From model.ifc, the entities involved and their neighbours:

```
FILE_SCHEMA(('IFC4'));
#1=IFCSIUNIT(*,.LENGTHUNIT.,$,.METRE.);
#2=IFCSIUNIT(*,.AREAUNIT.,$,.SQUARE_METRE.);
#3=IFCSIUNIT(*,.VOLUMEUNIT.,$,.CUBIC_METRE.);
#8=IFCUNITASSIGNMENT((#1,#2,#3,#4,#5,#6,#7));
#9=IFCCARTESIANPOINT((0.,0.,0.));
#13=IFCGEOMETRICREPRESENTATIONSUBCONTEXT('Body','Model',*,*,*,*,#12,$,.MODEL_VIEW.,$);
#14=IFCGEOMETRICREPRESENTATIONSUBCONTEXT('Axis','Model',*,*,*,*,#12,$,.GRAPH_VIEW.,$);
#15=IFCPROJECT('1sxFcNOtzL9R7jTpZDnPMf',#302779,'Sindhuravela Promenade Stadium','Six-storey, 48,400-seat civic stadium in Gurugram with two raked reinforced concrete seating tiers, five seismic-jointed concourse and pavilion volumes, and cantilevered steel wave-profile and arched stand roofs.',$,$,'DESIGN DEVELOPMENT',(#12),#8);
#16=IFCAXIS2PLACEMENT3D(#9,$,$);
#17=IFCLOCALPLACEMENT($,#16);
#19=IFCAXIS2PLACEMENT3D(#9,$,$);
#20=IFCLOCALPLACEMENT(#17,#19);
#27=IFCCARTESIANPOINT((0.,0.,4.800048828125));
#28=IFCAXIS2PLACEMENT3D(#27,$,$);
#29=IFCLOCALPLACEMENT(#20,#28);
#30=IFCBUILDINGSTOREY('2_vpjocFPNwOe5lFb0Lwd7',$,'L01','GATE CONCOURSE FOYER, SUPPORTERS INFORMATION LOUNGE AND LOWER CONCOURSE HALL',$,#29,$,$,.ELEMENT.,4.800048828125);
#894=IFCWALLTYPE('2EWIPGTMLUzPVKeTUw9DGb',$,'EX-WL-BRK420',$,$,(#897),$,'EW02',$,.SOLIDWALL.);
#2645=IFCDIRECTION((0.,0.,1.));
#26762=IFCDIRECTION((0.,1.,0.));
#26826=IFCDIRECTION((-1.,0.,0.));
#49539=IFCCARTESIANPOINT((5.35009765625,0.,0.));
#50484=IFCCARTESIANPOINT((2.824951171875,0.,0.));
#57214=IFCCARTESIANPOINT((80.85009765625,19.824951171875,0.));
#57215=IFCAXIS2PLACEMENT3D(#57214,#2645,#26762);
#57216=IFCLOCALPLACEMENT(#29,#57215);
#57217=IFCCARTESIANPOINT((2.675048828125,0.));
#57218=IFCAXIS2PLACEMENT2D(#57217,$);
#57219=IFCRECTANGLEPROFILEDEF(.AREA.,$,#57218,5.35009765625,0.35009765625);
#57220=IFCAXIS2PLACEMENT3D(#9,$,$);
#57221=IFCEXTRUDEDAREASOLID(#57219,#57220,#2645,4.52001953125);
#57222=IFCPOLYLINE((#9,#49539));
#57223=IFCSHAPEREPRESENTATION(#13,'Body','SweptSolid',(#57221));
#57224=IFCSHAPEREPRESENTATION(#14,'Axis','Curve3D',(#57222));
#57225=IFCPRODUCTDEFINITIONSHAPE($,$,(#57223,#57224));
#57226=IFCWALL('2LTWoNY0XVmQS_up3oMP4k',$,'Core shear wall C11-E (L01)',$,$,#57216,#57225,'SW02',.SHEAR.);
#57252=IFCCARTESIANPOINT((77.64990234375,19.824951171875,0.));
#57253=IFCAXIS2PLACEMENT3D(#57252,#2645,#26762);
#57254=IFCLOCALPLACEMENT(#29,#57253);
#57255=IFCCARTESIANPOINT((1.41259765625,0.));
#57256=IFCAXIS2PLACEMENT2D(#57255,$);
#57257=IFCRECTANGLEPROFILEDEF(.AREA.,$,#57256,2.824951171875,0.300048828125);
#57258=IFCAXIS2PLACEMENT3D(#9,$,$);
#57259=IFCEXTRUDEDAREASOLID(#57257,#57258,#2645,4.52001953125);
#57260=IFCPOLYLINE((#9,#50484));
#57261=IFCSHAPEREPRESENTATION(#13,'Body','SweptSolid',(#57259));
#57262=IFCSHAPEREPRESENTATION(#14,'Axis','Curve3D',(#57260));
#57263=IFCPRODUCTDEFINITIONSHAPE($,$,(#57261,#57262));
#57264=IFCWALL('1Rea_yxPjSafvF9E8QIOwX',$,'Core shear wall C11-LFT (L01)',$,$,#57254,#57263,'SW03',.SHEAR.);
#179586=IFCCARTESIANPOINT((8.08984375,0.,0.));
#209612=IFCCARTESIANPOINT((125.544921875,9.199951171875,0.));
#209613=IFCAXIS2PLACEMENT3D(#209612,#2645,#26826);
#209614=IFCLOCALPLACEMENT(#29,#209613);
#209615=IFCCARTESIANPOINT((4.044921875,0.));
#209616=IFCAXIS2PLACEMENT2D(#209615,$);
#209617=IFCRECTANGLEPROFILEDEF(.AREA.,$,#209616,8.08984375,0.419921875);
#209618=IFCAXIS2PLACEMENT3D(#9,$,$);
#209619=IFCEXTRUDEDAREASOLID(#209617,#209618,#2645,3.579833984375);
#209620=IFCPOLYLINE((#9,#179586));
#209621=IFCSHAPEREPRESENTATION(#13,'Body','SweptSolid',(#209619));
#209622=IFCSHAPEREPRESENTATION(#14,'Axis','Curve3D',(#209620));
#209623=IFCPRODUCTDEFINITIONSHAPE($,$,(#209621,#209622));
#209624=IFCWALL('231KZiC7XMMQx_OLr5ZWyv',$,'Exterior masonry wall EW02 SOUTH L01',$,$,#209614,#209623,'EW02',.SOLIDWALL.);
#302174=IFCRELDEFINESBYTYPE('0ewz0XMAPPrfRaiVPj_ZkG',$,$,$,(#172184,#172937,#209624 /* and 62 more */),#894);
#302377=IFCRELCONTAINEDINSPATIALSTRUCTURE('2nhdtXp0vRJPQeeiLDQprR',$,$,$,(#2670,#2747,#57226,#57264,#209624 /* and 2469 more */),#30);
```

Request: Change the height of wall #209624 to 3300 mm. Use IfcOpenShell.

```python
import ifcopenshell
import ifcopenshell.geom
import ifcopenshell.util.representation
import ifcopenshell.util.shape
import ifcopenshell.util.unit

model = ifcopenshell.open("model.ifc")
unit_scale = ifcopenshell.util.unit.calculate_unit_scale(model)
settings = ifcopenshell.geom.settings()


def volume(element):
    """Net volume in cubic metres, openings subtracted."""
    shape = ifcopenshell.geom.create_shape(settings, element)
    return ifcopenshell.util.shape.get_volume(shape.geometry)


wall = model.by_id(209624)
before = volume(wall)

body = ifcopenshell.util.representation.get_representation(wall, "Model", "Body")
solid = body.Items[0]
old_height = solid.Depth
solid.Depth = 3.3 / unit_scale
after = volume(wall)

print(f"height {old_height:g} -> {solid.Depth:g}, volume {before:.3f} -> {after:.3f} m3")

model.write("model_rev.ifc")
```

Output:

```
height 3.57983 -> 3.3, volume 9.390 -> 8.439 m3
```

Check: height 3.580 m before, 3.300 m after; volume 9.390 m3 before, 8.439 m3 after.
